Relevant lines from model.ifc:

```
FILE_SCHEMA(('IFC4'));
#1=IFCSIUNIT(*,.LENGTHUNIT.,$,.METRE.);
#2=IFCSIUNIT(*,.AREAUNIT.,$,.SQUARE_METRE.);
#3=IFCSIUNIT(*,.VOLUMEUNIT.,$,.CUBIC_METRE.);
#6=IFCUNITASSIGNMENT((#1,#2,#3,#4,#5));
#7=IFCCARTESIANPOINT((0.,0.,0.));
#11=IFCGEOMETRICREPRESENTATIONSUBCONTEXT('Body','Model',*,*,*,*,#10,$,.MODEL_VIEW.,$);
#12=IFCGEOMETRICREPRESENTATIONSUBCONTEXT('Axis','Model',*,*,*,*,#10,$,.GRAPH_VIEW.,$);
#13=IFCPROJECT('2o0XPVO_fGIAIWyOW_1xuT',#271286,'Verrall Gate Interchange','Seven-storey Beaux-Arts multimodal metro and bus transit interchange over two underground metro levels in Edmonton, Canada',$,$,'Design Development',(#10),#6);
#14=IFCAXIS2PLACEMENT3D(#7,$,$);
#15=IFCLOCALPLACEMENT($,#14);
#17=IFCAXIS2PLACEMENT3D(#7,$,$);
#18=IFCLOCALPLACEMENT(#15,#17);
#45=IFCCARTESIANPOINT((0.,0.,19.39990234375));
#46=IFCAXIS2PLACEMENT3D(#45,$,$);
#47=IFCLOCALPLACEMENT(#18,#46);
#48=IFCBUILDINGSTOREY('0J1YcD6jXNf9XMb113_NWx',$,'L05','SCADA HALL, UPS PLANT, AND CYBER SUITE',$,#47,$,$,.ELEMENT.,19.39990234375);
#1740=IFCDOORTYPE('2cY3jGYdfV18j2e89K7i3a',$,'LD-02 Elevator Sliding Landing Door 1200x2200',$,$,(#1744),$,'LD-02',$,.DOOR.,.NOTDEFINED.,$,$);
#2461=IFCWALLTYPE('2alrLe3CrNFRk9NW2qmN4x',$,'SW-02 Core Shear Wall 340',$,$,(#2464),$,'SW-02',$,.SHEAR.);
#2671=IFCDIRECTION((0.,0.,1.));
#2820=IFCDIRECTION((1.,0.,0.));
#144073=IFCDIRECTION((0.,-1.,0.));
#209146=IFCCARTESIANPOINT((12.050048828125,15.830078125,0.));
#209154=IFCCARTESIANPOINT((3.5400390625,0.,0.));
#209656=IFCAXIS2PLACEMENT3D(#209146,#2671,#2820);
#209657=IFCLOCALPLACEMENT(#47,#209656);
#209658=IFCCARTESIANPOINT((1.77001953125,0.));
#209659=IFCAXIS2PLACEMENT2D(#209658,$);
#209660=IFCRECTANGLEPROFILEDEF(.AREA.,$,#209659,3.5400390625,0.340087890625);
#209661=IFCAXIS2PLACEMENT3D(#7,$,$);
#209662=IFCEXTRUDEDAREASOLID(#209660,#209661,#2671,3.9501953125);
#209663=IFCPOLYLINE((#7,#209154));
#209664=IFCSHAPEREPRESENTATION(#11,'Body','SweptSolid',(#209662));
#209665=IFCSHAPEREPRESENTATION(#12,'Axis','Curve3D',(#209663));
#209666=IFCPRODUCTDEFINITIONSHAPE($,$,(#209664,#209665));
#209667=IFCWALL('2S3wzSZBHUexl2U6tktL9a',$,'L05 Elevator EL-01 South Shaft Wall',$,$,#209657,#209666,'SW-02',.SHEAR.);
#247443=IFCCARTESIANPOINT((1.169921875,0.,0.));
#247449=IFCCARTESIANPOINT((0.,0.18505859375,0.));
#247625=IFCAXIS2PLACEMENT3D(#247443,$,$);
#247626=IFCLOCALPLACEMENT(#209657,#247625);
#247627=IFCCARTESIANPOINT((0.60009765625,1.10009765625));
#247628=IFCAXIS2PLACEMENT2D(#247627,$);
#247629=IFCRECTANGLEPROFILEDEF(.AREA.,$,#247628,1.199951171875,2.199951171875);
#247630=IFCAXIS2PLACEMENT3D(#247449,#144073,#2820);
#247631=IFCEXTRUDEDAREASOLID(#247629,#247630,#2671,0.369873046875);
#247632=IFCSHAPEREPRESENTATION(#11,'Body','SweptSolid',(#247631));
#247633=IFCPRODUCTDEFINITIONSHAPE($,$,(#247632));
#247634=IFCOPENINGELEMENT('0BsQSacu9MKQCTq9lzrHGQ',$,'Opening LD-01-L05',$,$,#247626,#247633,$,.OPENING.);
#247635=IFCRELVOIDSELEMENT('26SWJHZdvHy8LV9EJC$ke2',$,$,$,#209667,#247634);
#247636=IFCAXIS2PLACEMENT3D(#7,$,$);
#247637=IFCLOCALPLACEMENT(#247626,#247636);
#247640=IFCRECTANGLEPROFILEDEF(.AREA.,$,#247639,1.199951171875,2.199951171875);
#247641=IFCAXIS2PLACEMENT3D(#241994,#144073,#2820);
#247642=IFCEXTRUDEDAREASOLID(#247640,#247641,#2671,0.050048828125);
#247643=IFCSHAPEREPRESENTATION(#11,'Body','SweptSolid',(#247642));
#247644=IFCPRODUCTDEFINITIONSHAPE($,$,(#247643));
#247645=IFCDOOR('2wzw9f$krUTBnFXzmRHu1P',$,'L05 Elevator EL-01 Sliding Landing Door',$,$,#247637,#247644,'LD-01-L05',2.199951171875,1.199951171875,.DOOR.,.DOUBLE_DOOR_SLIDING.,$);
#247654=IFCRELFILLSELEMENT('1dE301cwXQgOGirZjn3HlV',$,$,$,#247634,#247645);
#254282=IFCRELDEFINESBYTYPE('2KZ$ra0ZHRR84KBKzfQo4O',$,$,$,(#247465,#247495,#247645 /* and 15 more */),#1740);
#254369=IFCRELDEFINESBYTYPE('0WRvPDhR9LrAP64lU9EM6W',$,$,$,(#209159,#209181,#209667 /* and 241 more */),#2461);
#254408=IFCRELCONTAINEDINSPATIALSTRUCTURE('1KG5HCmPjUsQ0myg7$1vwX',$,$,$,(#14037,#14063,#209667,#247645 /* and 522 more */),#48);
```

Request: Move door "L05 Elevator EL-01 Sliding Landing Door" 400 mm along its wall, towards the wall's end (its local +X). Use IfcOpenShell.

```python
import ifcopenshell
import ifcopenshell.api.geometry
import ifcopenshell.util.placement
import ifcopenshell.util.unit

model = ifcopenshell.open("model.ifc")
unit_scale = ifcopenshell.util.unit.calculate_unit_scale(model)

door = model.by_guid("2wzw9f$krUTBnFXzmRHu1P")
opening = door.FillsVoids[0].RelatingOpeningElement
wall = opening.VoidsElements[0].RelatingBuildingElement

wall_matrix = ifcopenshell.util.placement.get_local_placement(wall.ObjectPlacement)
shift = wall_matrix[:3, 0] * 0.4 / unit_scale
before = ifcopenshell.util.placement.get_local_placement(door.ObjectPlacement)[:3, 3].copy()

# The door is placed relative to its opening, so it follows when the opening moves.
matrix = ifcopenshell.util.placement.get_local_placement(opening.ObjectPlacement)
matrix[:3, 3] += shift
ifcopenshell.api.geometry.edit_object_placement(
    model, product=opening, matrix=matrix, is_si=False, should_transform_children=True
)

after = ifcopenshell.util.placement.get_local_placement(door.ObjectPlacement)[:3, 3]
print("door moved by", (after - before).round(3) + 0.0)

model.write("model_edited.ifc")
```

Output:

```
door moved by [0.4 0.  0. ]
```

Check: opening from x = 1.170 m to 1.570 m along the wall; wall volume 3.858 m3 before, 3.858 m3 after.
